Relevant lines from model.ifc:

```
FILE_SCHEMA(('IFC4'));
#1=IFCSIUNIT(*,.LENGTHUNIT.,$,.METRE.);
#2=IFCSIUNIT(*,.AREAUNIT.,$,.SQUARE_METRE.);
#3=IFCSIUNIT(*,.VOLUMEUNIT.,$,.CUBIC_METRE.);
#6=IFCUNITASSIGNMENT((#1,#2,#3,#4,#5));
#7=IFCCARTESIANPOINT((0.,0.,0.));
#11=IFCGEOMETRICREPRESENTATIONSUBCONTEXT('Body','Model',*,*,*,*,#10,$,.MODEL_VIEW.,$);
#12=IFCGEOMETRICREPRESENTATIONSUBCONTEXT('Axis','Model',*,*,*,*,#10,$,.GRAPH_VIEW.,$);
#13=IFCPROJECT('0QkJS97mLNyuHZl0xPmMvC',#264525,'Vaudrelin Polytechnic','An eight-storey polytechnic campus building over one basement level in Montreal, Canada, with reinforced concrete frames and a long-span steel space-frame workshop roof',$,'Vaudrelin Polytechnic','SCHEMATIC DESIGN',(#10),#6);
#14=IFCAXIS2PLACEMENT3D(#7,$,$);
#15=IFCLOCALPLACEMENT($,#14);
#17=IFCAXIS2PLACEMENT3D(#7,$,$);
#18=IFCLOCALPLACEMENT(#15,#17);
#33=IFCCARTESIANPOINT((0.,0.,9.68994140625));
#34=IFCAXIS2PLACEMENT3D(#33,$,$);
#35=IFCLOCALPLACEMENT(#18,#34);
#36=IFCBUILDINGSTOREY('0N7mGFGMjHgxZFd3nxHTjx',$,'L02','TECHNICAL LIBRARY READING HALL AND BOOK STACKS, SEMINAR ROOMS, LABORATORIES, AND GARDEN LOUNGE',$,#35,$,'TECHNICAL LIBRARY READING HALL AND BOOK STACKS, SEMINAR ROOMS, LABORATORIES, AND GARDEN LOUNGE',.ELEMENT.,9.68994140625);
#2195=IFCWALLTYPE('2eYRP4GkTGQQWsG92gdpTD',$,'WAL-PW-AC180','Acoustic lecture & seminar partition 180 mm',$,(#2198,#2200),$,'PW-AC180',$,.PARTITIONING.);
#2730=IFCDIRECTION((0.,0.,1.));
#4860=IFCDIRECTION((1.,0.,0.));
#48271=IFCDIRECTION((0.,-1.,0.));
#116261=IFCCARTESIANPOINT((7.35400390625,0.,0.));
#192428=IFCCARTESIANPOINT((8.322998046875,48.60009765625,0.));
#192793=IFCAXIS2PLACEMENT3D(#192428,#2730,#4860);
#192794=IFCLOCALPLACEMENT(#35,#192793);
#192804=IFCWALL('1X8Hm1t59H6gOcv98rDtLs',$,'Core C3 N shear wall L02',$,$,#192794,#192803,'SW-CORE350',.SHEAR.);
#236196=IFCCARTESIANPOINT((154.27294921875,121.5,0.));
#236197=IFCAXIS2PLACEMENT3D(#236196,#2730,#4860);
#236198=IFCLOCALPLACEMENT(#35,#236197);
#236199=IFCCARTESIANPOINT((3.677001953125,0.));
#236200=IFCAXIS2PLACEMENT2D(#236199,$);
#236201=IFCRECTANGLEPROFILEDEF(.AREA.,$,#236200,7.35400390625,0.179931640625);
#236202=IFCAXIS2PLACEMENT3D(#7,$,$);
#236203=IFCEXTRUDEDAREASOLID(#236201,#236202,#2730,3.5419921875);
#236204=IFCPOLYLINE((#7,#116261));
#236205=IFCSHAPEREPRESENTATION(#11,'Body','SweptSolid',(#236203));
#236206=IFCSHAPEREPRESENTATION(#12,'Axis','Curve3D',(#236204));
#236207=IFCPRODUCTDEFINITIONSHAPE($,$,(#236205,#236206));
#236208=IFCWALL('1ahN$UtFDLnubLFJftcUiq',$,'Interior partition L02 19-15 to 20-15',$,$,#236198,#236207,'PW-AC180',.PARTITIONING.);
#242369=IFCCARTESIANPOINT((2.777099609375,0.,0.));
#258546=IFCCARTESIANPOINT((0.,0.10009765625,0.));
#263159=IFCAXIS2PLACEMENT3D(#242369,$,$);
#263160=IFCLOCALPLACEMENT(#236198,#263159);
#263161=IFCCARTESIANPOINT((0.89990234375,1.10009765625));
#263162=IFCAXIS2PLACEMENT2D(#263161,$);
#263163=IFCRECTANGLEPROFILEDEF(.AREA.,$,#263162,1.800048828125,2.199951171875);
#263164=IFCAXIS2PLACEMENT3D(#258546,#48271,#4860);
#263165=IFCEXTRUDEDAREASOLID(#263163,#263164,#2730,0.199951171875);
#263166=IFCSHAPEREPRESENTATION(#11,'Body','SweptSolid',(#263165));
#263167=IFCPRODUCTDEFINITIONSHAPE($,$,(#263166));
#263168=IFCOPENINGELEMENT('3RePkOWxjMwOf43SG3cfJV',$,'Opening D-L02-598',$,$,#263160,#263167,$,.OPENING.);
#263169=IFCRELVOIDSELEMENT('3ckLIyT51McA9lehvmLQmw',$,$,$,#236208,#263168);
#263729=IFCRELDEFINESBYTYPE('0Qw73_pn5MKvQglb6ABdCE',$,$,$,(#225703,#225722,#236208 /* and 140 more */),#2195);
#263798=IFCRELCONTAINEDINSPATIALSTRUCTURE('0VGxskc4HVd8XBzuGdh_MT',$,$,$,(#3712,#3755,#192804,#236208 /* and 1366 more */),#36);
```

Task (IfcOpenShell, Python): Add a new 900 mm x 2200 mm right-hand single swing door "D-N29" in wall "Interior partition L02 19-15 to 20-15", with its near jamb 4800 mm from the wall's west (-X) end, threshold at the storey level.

```python
import numpy as np
import ifcopenshell
import ifcopenshell.api.feature
import ifcopenshell.api.geometry
import ifcopenshell.api.root
import ifcopenshell.api.spatial
import ifcopenshell.geom
import ifcopenshell.util.element
import ifcopenshell.util.placement
import ifcopenshell.util.representation
import ifcopenshell.util.shape
import ifcopenshell.util.unit

model = ifcopenshell.open("model.ifc")
unit_scale = ifcopenshell.util.unit.calculate_unit_scale(model)
settings = ifcopenshell.geom.settings()


def volume(element):
    """Net volume in cubic metres, openings subtracted."""
    shape = ifcopenshell.geom.create_shape(settings, element)
    return ifcopenshell.util.shape.get_volume(shape.geometry)


wall = model.by_guid("1ahN$UtFDLnubLFJftcUiq")
storey = ifcopenshell.util.element.get_container(wall, ifc_class="IfcBuildingStorey")
context = ifcopenshell.util.representation.get_context(model, "Model", "Body", "MODEL_VIEW")
before = volume(wall)

width, height, from_end, sill = 0.9, 2.2, 4.8, 0.0  # metres

# The wall runs along its own X axis, and the end named is its -X end.
wall_shape = ifcopenshell.geom.create_shape(settings, wall)
x, y, z = ifcopenshell.util.shape.get_vertices(wall_shape.geometry).T
start = x.min() + from_end
face, thickness = float(y.min()), float(y.max() - y.min())
wall_matrix = ifcopenshell.util.placement.get_local_placement(wall.ObjectPlacement)
level = ifcopenshell.util.placement.get_local_placement(storey.ObjectPlacement)[2, 3]


def in_wall(x, y):
    """Placement at x, y metres in the wall's axes, at sill height."""
    matrix = wall_matrix.copy()
    matrix[:, 3] = wall_matrix @ np.array([x / unit_scale, y / unit_scale, 0.0, 1.0])
    matrix[2, 3] = level + sill / unit_scale
    return matrix


# Opening: a box that overshoots both wall faces by 50 mm.
opening = ifcopenshell.api.root.create_entity(model, ifc_class="IfcOpeningElement", predefined_type="OPENING")
box = ifcopenshell.api.geometry.add_wall_representation(
    model, context=context, length=width, height=height, thickness=thickness + 0.1
)
ifcopenshell.api.geometry.assign_representation(model, product=opening, representation=box)
ifcopenshell.api.geometry.edit_object_placement(model, product=opening, matrix=in_wall(start, face - 0.05), is_si=False)
ifcopenshell.api.feature.add_feature(model, feature=opening, element=wall)

door = ifcopenshell.api.root.create_entity(model, ifc_class="IfcDoor", name="D-N29", predefined_type="DOOR")
door.OverallWidth, door.OverallHeight = width / unit_scale, height / unit_scale
door.OperationType = "SINGLE_SWING_RIGHT"
body = ifcopenshell.api.geometry.add_door_representation(
    model,
    context=context,
    overall_width=door.OverallWidth,
    overall_height=door.OverallHeight,
    operation_type="SINGLE_SWING_RIGHT",
    lining_properties={"LiningDepth": thickness / unit_scale, "ThresholdDepth": thickness / unit_scale},
)
ifcopenshell.api.geometry.assign_representation(model, product=door, representation=body)
ifcopenshell.api.spatial.assign_container(model, products=[door], relating_structure=storey)
ifcopenshell.api.feature.add_filling(model, opening=opening, element=door)

# The lining spans the wall, so the door starts at the wall face.
ifcopenshell.api.geometry.edit_object_placement(model, product=door, matrix=in_wall(start, face), is_si=False)

after = volume(wall)

print(f"wall volume {before:.3f} -> {after:.3f} m3")

model.write("model-out.ifc")
```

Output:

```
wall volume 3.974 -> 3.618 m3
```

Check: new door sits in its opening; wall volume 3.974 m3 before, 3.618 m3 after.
